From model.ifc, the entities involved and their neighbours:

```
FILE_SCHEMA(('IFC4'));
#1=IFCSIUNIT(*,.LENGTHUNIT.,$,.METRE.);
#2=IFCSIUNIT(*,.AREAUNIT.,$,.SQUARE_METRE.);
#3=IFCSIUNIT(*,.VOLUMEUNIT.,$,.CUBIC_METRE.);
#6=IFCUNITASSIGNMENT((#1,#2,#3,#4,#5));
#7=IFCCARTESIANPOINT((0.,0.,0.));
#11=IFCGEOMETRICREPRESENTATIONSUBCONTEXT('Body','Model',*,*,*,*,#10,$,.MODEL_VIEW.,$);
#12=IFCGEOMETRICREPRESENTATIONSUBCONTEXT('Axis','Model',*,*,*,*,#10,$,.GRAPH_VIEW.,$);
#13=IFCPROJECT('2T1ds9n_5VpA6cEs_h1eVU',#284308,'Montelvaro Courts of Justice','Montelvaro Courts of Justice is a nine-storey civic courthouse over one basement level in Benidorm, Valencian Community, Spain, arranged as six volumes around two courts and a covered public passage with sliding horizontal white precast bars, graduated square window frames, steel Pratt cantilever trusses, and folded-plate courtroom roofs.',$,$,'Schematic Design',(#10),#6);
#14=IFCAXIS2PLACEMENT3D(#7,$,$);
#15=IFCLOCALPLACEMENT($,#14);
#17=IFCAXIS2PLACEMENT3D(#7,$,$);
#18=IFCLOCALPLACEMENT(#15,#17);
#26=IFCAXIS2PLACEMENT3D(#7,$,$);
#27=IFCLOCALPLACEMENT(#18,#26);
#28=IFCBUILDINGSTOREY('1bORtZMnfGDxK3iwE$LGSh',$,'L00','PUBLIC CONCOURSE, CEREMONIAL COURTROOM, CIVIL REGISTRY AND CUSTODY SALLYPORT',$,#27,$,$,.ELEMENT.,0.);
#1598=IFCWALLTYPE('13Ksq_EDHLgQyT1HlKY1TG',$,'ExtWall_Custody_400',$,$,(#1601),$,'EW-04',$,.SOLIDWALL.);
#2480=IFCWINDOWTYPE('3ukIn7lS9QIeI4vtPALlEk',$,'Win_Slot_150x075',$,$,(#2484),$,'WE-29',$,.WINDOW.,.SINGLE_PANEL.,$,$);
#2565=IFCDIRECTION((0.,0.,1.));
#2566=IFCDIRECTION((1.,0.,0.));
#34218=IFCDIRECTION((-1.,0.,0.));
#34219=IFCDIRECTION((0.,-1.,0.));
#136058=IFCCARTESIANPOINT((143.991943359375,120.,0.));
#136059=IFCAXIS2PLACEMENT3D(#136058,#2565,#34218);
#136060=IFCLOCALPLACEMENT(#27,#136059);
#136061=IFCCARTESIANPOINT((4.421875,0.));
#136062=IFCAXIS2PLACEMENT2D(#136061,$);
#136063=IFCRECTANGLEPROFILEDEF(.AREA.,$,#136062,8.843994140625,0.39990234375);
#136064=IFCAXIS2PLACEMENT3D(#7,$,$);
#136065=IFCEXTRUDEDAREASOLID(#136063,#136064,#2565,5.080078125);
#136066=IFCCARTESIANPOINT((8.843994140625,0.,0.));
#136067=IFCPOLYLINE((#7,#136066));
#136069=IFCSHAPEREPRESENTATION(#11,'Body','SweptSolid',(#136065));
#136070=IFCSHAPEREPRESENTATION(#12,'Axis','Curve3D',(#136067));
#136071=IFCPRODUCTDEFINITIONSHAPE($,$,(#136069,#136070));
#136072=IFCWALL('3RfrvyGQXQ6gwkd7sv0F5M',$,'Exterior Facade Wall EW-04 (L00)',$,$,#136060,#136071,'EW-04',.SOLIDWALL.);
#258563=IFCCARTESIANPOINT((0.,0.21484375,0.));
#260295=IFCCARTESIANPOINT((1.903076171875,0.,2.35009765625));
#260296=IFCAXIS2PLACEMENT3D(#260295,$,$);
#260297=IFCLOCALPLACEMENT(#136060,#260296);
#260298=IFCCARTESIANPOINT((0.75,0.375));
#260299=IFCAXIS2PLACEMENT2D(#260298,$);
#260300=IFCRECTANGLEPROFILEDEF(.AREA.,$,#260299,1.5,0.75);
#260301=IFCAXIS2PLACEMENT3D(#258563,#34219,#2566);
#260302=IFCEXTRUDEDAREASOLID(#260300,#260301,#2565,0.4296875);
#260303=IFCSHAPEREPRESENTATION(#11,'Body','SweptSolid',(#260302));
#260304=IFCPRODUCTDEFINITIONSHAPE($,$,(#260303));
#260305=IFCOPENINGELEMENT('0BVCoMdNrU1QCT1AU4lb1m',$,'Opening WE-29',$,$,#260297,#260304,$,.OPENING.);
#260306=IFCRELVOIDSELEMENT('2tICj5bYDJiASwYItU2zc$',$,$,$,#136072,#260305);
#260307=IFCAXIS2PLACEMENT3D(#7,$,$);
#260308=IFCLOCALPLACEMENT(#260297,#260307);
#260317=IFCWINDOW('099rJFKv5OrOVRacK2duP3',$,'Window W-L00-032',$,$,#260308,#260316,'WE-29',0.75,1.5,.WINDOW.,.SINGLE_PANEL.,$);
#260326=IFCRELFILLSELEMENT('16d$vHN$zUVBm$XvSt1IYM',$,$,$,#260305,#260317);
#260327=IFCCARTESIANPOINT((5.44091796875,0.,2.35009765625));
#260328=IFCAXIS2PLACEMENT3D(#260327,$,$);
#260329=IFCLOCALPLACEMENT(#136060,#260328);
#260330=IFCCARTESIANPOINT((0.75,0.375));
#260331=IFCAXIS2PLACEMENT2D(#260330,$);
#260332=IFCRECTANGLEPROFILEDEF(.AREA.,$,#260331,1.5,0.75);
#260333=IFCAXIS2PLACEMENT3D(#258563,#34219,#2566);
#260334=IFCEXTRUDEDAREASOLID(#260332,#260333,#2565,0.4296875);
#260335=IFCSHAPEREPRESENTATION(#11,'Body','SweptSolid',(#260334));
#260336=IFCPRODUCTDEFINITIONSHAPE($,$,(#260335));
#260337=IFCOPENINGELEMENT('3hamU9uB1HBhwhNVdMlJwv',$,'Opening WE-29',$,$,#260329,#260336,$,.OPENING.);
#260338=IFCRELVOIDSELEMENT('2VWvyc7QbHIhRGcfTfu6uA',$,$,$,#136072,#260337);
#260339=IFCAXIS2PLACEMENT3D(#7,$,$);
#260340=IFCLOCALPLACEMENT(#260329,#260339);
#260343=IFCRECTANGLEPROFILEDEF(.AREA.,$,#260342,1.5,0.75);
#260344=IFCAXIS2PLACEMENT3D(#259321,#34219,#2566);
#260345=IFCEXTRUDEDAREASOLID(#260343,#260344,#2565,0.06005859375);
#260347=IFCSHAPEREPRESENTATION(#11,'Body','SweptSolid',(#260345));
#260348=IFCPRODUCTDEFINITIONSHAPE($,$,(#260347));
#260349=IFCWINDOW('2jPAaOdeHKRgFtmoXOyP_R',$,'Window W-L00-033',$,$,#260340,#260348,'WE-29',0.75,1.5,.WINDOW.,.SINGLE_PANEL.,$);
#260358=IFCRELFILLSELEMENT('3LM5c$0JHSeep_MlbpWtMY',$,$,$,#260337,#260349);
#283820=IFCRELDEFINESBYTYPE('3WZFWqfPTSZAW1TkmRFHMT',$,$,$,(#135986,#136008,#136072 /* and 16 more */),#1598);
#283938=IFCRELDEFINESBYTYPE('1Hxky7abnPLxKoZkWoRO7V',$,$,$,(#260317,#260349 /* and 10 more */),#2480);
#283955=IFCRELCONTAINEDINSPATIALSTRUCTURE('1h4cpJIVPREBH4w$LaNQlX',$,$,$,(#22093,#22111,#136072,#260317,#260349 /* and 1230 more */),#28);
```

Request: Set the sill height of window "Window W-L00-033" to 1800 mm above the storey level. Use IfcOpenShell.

```python
import numpy as np
import ifcopenshell
import ifcopenshell.api.geometry
import ifcopenshell.geom
import ifcopenshell.util.element
import ifcopenshell.util.placement
import ifcopenshell.util.shape
import ifcopenshell.util.unit

model = ifcopenshell.open("model.ifc")
unit_scale = ifcopenshell.util.unit.calculate_unit_scale(model)

window = model.by_guid("2jPAaOdeHKRgFtmoXOyP_R")
opening = window.FillsVoids[0].RelatingOpeningElement
storey = ifcopenshell.util.element.get_container(window, ifc_class="IfcBuildingStorey")
level = ifcopenshell.util.placement.get_local_placement(storey.ObjectPlacement)[2, 3]

# The opening's origin need not be at the sill, so measure its lowest point.
shape = ifcopenshell.geom.create_shape(ifcopenshell.geom.settings(), opening)
bottom = ifcopenshell.util.shape.get_shape_bottom_elevation(shape, shape.geometry) / unit_scale
dz = level + 1.8 / unit_scale - bottom

shift = np.array([0.0, 0.0, dz])
# The window is placed relative to its opening, so it follows when the opening moves.
matrix = ifcopenshell.util.placement.get_local_placement(opening.ObjectPlacement)
matrix[:3, 3] += shift
ifcopenshell.api.geometry.edit_object_placement(
    model, product=opening, matrix=matrix, is_si=False, should_transform_children=True
)

print(f"moved by {dz * unit_scale:+.3f} m")

model.write("model_v2.ifc")
```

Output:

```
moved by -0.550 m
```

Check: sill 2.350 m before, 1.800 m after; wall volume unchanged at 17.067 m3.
